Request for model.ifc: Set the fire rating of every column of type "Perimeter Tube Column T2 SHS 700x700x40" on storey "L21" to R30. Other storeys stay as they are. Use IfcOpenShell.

First a look at what the model holds.

```python
import ifcopenshell
import ifcopenshell.util.element

model = ifcopenshell.open("model.ifc")
print(model.schema)
storey = next(s for s in model.by_type("IfcBuildingStorey") if s.Name == "L21")
columns = [e for e in ifcopenshell.util.element.get_decomposition(storey) if e.is_a("IfcColumn")]
seen = {}
for e in columns:
    element_type = ifcopenshell.util.element.get_type(e)
    key = (element_type.Name if element_type != e and element_type else None, ifcopenshell.util.element.get_pset(e, "Pset_ColumnCommon", "FireRating"))
    seen[key] = seen.get(key, 0) + 1
for (name, value), count in sorted(seen.items(), key=str):
    print(count, "x", name, "|", value)
```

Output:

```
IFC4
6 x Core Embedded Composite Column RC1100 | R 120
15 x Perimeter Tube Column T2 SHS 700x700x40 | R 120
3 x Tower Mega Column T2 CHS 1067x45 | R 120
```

```python
import ifcopenshell
import ifcopenshell.api.pset
import ifcopenshell.util.element

model = ifcopenshell.open("model.ifc")

storey = next(s for s in model.by_type("IfcBuildingStorey") if s.Name == "L21")
columns = [e for e in ifcopenshell.util.element.get_decomposition(storey) if e.is_a("IfcColumn")]

count = 0
for e in columns:
    element_type = ifcopenshell.util.element.get_type(e)
    if element_type in (None, e) or element_type.Name != "Perimeter Tube Column T2 SHS 700x700x40":
        continue
    found = ifcopenshell.util.element.get_pset(e, "Pset_ColumnCommon", should_inherit=False)
    if found:
        pset = model.by_id(found["id"])
        if len(ifcopenshell.util.element.get_elements_by_pset(pset)) > 1:
            pset = ifcopenshell.api.pset.unshare_pset(model, products=[e], pset=pset)[0]
    else:
        pset = ifcopenshell.api.pset.add_pset(model, product=e, name="Pset_ColumnCommon")
    ifcopenshell.api.pset.edit_pset(model, pset=pset, properties={"FireRating": "R30"})
    count += 1

print(count, "columns updated")

model.write("model_edited.ifc")
```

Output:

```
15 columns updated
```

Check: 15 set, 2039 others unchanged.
